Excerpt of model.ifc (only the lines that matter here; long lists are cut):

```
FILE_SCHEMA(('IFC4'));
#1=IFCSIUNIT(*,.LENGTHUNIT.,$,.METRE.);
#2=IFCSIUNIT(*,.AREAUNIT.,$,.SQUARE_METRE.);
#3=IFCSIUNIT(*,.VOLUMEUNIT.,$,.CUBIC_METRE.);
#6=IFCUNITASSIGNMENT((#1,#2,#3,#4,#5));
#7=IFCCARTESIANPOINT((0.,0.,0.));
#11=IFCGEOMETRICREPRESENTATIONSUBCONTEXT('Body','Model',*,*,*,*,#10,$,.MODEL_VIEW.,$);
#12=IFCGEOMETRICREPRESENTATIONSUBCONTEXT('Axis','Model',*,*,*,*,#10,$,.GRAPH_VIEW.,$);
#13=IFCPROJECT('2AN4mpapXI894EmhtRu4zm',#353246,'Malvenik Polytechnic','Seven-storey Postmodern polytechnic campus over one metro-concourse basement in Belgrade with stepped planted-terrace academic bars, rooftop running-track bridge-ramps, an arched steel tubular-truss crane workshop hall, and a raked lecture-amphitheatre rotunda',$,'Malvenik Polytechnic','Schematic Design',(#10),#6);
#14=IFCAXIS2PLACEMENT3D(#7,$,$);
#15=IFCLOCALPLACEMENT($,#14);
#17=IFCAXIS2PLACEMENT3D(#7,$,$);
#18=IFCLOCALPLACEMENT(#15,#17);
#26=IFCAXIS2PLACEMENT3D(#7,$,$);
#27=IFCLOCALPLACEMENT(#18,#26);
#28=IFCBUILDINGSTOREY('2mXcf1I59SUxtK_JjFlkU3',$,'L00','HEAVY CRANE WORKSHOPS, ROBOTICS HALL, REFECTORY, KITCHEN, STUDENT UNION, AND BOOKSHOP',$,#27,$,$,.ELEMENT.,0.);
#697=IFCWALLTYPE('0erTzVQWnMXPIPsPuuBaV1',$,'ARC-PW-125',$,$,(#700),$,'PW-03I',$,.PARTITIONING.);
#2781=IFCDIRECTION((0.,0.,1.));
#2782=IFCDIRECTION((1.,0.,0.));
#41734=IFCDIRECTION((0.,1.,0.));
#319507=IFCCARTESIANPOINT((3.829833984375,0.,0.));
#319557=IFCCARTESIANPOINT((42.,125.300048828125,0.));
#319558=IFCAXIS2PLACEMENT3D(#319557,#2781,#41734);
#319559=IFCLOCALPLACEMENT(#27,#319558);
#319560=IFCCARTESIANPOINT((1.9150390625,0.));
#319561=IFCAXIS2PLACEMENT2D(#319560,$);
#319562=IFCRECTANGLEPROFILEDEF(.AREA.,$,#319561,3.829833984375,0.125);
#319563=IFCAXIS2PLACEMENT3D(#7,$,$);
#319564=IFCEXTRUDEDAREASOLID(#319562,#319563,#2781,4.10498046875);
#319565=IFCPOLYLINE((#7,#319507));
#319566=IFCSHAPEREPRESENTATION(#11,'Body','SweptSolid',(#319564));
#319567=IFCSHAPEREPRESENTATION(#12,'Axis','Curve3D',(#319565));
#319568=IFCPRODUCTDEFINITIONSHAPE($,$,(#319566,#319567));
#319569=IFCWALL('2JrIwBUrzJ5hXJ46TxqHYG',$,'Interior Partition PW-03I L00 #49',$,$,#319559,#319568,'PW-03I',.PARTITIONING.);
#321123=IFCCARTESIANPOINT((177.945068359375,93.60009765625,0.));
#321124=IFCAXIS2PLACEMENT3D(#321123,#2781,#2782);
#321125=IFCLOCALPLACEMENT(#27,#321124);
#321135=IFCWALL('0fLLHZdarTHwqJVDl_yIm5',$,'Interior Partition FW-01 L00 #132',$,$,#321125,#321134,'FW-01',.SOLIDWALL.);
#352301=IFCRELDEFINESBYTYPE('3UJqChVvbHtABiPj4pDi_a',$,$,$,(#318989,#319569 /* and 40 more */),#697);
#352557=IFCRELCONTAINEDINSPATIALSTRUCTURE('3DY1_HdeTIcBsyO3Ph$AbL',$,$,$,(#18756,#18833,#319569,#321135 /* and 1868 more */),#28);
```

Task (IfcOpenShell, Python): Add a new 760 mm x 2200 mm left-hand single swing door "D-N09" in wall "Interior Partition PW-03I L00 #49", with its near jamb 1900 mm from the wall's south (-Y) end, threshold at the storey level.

```python
import numpy as np
import ifcopenshell
import ifcopenshell.api.feature
import ifcopenshell.api.geometry
import ifcopenshell.api.root
import ifcopenshell.api.spatial
import ifcopenshell.geom
import ifcopenshell.util.element
import ifcopenshell.util.placement
import ifcopenshell.util.representation
import ifcopenshell.util.shape
import ifcopenshell.util.unit

model = ifcopenshell.open("model.ifc")
unit_scale = ifcopenshell.util.unit.calculate_unit_scale(model)
settings = ifcopenshell.geom.settings()


def volume(element):
    """Net volume in cubic metres, openings subtracted."""
    shape = ifcopenshell.geom.create_shape(settings, element)
    return ifcopenshell.util.shape.get_volume(shape.geometry)


wall = model.by_guid("2JrIwBUrzJ5hXJ46TxqHYG")
storey = ifcopenshell.util.element.get_container(wall, ifc_class="IfcBuildingStorey")
context = ifcopenshell.util.representation.get_context(model, "Model", "Body", "MODEL_VIEW")
before = volume(wall)

width, height, from_end, sill = 0.76, 2.2, 1.9, 0.0  # metres

# The wall runs along its own X axis, and the end named is its -X end.
wall_shape = ifcopenshell.geom.create_shape(settings, wall)
x, y, z = ifcopenshell.util.shape.get_vertices(wall_shape.geometry).T
start = x.min() + from_end
face, thickness = float(y.min()), float(y.max() - y.min())
wall_matrix = ifcopenshell.util.placement.get_local_placement(wall.ObjectPlacement)
level = ifcopenshell.util.placement.get_local_placement(storey.ObjectPlacement)[2, 3]


def in_wall(x, y):
    """Placement at x, y metres in the wall's axes, at sill height."""
    matrix = wall_matrix.copy()
    matrix[:, 3] = wall_matrix @ np.array([x / unit_scale, y / unit_scale, 0.0, 1.0])
    matrix[2, 3] = level + sill / unit_scale
    return matrix


# Opening: a box that overshoots both wall faces by 50 mm.
opening = ifcopenshell.api.root.create_entity(model, ifc_class="IfcOpeningElement", predefined_type="OPENING")
box = ifcopenshell.api.geometry.add_wall_representation(
    model, context=context, length=width, height=height, thickness=thickness + 0.1
)
ifcopenshell.api.geometry.assign_representation(model, product=opening, representation=box)
ifcopenshell.api.geometry.edit_object_placement(model, product=opening, matrix=in_wall(start, face - 0.05), is_si=False)
ifcopenshell.api.feature.add_feature(model, feature=opening, element=wall)

door = ifcopenshell.api.root.create_entity(model, ifc_class="IfcDoor", name="D-N09", predefined_type="DOOR")
door.OverallWidth, door.OverallHeight = width / unit_scale, height / unit_scale
door.OperationType = "SINGLE_SWING_LEFT"
body = ifcopenshell.api.geometry.add_door_representation(
    model,
    context=context,
    overall_width=door.OverallWidth,
    overall_height=door.OverallHeight,
    operation_type="SINGLE_SWING_LEFT",
    lining_properties={"LiningDepth": thickness / unit_scale, "ThresholdDepth": thickness / unit_scale},
)
ifcopenshell.api.geometry.assign_representation(model, product=door, representation=body)
ifcopenshell.api.spatial.assign_container(model, products=[door], relating_structure=storey)
ifcopenshell.api.feature.add_filling(model, opening=opening, element=door)

# The lining spans the wall, so the door starts at the wall face.
ifcopenshell.api.geometry.edit_object_placement(model, product=door, matrix=in_wall(start, face), is_si=False)

after = volume(wall)

print(f"wall volume {before:.3f} -> {after:.3f} m3")

model.write("model-out.ifc")
```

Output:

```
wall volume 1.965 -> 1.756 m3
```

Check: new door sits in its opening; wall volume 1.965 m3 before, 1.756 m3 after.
